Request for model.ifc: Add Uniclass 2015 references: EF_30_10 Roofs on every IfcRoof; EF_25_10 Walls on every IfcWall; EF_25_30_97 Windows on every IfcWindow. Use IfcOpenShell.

First a look at what the model holds.

```python
import ifcopenshell

model = ifcopenshell.open("model.ifc")
print(model.schema)
print("classifications:", [c.Name for c in model.by_type("IfcClassification")])
for ifc_class in ("IfcDoor", "IfcRoof", "IfcStair", "IfcWall", "IfcWindow"):
    print(ifc_class, len(model.by_type(ifc_class)))
```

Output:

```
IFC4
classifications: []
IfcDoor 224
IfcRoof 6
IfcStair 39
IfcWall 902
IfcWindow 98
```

```python
import ifcopenshell
import ifcopenshell.api.classification

model = ifcopenshell.open("model.ifc")

system = ifcopenshell.api.classification.add_classification(model, classification="Uniclass 2015")

codes = {
    "IfcRoof": ("EF_30_10", "Roofs"),
    "IfcWall": ("EF_25_10", "Walls"),
    "IfcWindow": ("EF_25_30_97", "Windows"),
}
for ifc_class, (code, name) in codes.items():
    products = model.by_type(ifc_class)
    ifcopenshell.api.classification.add_reference(
        model, products=products, classification=system, identification=code, name=name
    )
    print(code, len(products))

model.write("model_v2.ifc")
```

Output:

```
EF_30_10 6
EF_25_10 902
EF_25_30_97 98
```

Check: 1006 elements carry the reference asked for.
